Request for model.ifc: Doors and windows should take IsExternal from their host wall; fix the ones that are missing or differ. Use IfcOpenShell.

First a look at what the model holds.

```python
import ifcopenshell
import ifcopenshell.util.element

model = ifcopenshell.open("model.ifc")
print(model.schema)
seen = {}
for e in model.by_type("IfcDoor") + model.by_type("IfcWindow"):
    if not e.FillsVoids:
        continue
    host = e.FillsVoids[0].RelatingOpeningElement.VoidsElements[0].RelatingBuildingElement
    own = ifcopenshell.util.element.get_pset(e, f"Pset_{e.is_a()[3:].removesuffix('StandardCase')}Common", "IsExternal")
    wall = ifcopenshell.util.element.get_pset(host, "Pset_WallCommon", "IsExternal")
    seen[e.is_a(), own, wall] = seen.get((e.is_a(), own, wall), 0) + 1
for (cls, own, wall), count in sorted(seen.items(), key=str):
    print(count, cls, "IsExternal:", own, "| host wall:", wall)
```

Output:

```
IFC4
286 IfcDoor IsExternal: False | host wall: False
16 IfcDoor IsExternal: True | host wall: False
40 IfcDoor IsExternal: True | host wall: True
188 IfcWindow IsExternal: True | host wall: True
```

```python
import ifcopenshell
import ifcopenshell.api.pset
import ifcopenshell.util.element

model = ifcopenshell.open("model.ifc")

count = 0
for ifc_class, pset_name in (("IfcDoor", "Pset_DoorCommon"), ("IfcWindow", "Pset_WindowCommon")):
    for e in model.by_type(ifc_class):
        if not e.FillsVoids:
            continue
        host = e.FillsVoids[0].RelatingOpeningElement.VoidsElements[0].RelatingBuildingElement
        external = ifcopenshell.util.element.get_pset(host, "Pset_WallCommon", "IsExternal")
        if external is None or ifcopenshell.util.element.get_pset(e, pset_name, "IsExternal") == external:
            continue
        pset = ifcopenshell.api.pset.add_pset(model, product=e, name=pset_name)
        ifcopenshell.api.pset.edit_pset(model, pset=pset, properties={"IsExternal": external})
        count += 1

print(count, "updated")

model.write("model_updated.ifc")
```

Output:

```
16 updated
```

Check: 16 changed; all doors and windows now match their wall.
